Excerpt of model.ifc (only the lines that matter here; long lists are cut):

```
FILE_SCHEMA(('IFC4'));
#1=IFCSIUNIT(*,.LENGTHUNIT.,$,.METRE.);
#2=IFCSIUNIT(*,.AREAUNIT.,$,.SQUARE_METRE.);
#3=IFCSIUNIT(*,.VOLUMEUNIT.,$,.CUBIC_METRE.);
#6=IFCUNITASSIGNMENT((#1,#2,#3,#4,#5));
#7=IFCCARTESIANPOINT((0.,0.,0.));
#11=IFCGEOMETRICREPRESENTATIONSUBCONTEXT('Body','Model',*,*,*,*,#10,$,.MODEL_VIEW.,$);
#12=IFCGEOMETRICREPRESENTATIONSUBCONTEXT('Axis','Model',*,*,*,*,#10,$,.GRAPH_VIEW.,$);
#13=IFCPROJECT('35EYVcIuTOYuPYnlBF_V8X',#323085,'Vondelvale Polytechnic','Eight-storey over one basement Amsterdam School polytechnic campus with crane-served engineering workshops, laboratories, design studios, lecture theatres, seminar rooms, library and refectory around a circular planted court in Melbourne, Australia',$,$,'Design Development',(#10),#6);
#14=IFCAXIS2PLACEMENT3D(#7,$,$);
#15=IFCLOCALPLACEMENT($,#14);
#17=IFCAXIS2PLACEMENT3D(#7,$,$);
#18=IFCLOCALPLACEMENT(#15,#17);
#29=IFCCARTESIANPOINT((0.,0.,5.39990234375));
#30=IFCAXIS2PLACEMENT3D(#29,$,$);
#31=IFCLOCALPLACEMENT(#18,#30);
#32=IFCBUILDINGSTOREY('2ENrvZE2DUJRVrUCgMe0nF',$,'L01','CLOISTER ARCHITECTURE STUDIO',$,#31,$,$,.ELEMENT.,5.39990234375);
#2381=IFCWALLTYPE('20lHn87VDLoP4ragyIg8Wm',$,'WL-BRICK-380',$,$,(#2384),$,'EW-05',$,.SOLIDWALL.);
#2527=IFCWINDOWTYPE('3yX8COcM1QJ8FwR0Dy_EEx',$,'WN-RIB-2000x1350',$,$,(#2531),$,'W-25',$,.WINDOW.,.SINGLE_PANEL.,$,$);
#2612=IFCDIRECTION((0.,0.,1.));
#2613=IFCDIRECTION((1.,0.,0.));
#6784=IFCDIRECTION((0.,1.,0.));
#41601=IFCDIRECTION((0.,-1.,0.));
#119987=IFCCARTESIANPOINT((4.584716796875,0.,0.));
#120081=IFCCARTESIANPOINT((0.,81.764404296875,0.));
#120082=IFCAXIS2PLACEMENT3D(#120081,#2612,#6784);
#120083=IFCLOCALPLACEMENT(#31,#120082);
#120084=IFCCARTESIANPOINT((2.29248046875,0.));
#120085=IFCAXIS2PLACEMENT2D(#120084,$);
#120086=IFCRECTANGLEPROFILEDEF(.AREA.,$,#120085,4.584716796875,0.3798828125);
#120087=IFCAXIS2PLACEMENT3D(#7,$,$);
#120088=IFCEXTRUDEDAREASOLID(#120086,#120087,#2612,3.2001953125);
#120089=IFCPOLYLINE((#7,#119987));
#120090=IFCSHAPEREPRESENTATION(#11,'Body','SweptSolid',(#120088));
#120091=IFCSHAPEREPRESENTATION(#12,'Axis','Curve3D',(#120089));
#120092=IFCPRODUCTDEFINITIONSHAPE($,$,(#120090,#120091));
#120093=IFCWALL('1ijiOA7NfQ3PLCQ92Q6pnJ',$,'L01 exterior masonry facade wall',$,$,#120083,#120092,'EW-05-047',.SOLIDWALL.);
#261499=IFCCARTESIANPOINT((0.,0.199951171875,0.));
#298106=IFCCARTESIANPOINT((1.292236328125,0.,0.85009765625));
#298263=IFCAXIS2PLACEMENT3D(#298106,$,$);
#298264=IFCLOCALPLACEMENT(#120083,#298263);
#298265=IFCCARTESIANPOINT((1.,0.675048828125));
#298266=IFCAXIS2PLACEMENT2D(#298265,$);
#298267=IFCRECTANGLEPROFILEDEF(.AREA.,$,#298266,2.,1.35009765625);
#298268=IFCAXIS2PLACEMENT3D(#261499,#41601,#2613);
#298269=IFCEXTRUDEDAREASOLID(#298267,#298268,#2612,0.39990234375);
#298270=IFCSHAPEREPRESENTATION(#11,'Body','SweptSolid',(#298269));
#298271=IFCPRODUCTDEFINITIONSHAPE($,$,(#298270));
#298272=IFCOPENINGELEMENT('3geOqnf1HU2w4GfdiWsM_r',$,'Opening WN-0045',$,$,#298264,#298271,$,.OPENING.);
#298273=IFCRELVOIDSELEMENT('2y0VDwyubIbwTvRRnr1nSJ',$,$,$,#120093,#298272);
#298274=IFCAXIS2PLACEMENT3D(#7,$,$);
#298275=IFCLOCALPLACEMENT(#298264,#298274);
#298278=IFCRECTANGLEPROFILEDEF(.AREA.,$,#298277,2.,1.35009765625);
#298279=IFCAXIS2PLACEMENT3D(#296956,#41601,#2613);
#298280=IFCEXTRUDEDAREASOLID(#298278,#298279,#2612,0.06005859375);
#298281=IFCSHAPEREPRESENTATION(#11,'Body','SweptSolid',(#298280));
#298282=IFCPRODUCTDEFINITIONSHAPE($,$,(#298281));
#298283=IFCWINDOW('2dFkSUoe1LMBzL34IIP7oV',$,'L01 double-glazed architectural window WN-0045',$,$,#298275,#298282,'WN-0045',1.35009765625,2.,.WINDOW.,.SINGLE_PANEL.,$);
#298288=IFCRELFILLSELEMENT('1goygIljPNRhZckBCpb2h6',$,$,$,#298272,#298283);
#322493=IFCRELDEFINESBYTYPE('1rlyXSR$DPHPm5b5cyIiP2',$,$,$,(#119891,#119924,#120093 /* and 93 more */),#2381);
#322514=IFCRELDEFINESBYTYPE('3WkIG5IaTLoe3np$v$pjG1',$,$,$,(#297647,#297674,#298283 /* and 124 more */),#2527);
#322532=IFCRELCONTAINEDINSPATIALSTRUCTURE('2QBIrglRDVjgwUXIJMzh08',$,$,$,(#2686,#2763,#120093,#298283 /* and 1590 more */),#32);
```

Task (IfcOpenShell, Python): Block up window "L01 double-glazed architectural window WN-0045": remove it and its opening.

```python
import ifcopenshell
import ifcopenshell.api.feature
import ifcopenshell.api.root
import ifcopenshell.geom
import ifcopenshell.util.shape

model = ifcopenshell.open("model.ifc")
settings = ifcopenshell.geom.settings()


def volume(element):
    """Net volume in cubic metres, openings subtracted."""
    shape = ifcopenshell.geom.create_shape(settings, element)
    return ifcopenshell.util.shape.get_volume(shape.geometry)


window = model.by_guid("2dFkSUoe1LMBzL34IIP7oV")
opening = window.FillsVoids[0].RelatingOpeningElement
wall = opening.VoidsElements[0].RelatingBuildingElement
before = volume(wall)

ifcopenshell.api.root.remove_product(model, product=window)
ifcopenshell.api.feature.remove_feature(model, feature=opening)

after = volume(wall)

print(f"wall volume {before:.3f} -> {after:.3f} m3")

model.write("model_updated.ifc")
```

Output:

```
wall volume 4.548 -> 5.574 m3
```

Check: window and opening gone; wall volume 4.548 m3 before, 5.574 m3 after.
